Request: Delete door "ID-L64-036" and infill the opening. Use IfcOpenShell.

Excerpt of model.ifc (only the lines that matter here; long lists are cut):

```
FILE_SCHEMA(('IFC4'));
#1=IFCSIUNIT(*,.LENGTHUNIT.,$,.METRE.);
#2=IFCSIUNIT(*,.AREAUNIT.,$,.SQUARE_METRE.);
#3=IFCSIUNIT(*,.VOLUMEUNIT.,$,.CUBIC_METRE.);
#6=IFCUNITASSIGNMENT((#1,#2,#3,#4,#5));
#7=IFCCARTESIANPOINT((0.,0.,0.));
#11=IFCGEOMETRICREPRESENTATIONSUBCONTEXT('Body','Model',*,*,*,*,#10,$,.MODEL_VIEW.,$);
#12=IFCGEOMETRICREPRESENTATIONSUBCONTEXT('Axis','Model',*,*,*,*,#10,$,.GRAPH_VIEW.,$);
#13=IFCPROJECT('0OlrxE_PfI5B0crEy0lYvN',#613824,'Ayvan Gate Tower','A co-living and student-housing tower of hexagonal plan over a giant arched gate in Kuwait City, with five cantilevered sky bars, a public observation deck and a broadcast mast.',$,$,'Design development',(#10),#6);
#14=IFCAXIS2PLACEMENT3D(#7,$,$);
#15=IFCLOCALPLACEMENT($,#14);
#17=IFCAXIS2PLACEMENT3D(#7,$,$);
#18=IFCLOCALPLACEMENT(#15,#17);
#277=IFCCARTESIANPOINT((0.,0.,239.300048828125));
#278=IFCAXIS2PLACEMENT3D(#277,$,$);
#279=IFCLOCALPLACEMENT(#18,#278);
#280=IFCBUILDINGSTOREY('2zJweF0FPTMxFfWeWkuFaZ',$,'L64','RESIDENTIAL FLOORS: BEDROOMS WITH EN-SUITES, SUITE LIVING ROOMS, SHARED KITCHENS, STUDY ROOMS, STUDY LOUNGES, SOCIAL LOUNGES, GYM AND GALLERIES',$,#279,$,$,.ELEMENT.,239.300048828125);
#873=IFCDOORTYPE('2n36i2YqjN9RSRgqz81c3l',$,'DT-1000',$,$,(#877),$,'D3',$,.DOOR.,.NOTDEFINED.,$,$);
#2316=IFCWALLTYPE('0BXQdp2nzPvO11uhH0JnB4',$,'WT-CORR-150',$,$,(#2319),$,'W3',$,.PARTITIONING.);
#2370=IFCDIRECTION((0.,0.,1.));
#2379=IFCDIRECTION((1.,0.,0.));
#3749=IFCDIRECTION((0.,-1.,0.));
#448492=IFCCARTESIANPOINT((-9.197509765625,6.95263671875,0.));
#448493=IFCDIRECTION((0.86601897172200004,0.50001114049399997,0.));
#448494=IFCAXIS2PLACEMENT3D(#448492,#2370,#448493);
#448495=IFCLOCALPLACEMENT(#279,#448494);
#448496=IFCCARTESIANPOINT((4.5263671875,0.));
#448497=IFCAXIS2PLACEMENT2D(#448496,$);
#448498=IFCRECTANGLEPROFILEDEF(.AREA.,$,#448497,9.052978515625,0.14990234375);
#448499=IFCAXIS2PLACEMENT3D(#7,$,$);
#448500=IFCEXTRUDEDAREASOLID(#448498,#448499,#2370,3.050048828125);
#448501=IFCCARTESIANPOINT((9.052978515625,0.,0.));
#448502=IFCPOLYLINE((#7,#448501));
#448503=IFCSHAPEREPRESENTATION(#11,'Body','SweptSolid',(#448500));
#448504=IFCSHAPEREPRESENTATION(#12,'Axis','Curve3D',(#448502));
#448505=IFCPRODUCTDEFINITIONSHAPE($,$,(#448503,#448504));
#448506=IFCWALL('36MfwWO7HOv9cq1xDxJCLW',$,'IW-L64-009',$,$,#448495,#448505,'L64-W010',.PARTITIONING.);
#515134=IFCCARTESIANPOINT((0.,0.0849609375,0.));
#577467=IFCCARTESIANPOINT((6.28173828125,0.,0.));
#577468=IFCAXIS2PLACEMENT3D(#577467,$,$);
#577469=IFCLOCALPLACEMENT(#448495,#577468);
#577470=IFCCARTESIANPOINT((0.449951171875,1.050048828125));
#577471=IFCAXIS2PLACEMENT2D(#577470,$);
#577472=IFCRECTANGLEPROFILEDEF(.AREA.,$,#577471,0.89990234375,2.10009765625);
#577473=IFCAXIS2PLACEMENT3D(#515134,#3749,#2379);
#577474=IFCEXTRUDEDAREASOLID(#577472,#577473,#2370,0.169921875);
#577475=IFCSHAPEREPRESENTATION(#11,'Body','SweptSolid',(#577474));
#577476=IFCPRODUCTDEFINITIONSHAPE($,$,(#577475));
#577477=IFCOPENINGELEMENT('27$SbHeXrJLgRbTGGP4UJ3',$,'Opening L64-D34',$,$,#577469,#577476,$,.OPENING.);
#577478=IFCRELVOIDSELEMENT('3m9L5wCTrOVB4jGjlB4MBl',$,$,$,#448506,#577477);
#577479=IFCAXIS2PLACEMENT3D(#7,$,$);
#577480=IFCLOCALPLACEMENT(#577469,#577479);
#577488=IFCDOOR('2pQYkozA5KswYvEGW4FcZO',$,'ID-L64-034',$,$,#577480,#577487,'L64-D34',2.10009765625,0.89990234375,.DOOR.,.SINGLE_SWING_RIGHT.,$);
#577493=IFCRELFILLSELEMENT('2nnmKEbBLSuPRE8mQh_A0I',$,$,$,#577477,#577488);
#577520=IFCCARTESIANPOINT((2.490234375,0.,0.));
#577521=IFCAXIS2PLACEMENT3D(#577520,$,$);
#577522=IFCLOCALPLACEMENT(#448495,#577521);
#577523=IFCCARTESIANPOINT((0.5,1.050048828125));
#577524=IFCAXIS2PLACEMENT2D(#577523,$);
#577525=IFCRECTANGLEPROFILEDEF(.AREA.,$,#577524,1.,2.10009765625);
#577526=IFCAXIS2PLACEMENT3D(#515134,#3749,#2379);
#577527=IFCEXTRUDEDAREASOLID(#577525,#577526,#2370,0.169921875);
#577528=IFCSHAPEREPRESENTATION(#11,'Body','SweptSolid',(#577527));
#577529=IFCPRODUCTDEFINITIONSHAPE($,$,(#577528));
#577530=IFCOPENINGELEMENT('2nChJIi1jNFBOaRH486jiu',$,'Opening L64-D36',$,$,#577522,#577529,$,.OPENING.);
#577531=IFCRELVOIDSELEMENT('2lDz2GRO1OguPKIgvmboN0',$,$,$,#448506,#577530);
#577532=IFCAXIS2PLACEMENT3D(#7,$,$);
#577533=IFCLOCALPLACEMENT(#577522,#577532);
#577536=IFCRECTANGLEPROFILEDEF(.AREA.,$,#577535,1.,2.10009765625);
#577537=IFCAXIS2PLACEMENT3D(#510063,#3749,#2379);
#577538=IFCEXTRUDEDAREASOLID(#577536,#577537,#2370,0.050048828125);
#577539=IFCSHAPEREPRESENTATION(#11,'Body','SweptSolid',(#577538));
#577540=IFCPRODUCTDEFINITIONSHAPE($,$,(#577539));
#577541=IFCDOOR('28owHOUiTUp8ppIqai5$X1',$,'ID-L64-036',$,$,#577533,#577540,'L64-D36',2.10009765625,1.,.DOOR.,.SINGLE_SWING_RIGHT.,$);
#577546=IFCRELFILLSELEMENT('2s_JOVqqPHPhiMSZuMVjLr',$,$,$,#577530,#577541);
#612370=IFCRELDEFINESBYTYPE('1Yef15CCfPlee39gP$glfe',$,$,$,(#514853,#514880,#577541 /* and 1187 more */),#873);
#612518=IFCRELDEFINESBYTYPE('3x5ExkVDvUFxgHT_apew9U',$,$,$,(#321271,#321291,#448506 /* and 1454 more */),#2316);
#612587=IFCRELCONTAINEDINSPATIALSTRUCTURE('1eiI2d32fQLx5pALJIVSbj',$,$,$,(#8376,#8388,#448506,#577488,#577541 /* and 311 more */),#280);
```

```python
import ifcopenshell
import ifcopenshell.api.feature
import ifcopenshell.api.root
import ifcopenshell.geom
import ifcopenshell.util.shape

model = ifcopenshell.open("model.ifc")
settings = ifcopenshell.geom.settings()


def volume(element):
    """Net volume in cubic metres, openings subtracted."""
    shape = ifcopenshell.geom.create_shape(settings, element)
    return ifcopenshell.util.shape.get_volume(shape.geometry)


door = model.by_id(577541)
opening = door.FillsVoids[0].RelatingOpeningElement
wall = opening.VoidsElements[0].RelatingBuildingElement
before = volume(wall)

ifcopenshell.api.root.remove_product(model, product=door)
ifcopenshell.api.feature.remove_feature(model, feature=opening)

after = volume(wall)

print(f"wall volume {before:.3f} -> {after:.3f} m3")

model.write("model_v2.ifc")
```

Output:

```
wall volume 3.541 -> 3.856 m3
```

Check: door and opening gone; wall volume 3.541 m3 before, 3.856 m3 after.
